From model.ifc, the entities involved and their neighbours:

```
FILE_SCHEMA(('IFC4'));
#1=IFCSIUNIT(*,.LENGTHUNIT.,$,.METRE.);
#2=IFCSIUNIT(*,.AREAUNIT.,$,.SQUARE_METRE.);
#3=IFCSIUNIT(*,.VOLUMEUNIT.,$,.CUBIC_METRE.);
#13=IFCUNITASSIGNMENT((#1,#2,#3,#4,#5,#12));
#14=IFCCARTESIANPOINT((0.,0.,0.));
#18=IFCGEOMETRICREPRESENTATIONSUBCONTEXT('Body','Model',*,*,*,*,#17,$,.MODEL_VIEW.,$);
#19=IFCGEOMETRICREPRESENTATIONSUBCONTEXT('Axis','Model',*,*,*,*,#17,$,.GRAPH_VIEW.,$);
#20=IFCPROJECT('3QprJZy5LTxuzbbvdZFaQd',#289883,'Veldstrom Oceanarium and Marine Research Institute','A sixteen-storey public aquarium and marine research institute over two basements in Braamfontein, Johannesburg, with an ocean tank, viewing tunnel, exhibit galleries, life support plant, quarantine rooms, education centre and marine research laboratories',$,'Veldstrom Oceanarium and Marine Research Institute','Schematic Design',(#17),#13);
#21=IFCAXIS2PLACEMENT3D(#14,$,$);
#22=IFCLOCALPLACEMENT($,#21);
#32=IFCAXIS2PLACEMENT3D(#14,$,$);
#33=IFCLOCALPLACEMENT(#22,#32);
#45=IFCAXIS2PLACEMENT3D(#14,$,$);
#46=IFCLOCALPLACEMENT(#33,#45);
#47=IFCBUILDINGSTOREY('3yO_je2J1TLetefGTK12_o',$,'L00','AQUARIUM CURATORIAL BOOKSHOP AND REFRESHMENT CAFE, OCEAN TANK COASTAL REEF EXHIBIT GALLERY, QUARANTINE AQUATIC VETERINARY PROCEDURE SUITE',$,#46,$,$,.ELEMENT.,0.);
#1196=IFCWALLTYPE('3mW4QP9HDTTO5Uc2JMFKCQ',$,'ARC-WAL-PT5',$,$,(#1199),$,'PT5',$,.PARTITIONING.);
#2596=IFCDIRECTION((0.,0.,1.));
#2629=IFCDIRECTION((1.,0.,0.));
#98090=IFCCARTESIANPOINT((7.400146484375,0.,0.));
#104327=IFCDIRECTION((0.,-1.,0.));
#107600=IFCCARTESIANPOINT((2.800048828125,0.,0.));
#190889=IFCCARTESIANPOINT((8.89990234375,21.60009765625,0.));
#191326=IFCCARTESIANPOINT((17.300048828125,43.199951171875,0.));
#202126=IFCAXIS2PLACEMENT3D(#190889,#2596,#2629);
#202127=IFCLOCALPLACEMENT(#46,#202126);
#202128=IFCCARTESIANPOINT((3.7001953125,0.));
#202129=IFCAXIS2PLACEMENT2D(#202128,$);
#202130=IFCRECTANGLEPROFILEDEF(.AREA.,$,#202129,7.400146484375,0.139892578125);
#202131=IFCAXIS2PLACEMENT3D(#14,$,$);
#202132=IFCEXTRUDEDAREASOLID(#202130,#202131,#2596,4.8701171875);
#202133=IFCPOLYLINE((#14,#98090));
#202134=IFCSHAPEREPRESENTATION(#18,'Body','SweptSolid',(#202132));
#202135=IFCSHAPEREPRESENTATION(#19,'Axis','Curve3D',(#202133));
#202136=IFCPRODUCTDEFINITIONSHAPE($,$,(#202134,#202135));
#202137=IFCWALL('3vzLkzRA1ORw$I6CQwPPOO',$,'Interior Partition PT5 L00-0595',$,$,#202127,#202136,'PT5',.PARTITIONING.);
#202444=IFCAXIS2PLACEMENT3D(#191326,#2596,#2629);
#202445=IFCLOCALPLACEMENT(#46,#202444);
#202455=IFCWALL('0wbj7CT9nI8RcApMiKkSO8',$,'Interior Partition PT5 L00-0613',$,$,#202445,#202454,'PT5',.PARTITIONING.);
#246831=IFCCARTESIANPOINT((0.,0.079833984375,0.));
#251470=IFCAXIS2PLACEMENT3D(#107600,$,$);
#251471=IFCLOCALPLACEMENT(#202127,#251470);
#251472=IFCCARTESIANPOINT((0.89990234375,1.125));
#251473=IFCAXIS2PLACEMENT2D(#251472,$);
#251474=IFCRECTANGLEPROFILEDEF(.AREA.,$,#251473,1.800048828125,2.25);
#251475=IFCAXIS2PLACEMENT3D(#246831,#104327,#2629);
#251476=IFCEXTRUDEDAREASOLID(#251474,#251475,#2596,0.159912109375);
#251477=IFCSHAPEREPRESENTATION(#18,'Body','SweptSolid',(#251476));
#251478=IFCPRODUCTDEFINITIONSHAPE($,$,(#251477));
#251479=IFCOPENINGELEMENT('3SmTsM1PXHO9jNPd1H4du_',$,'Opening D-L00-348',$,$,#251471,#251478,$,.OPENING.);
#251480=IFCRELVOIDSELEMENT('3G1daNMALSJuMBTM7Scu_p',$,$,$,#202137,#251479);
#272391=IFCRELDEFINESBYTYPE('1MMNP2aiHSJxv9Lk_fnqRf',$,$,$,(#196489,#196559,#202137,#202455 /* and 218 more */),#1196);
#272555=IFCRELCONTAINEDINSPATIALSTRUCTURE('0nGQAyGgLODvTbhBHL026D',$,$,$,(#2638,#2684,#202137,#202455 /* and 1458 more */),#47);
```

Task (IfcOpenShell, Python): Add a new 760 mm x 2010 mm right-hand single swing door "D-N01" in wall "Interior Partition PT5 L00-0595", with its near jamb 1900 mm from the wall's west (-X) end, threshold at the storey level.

```python
import numpy as np
import ifcopenshell
import ifcopenshell.api.feature
import ifcopenshell.api.geometry
import ifcopenshell.api.root
import ifcopenshell.api.spatial
import ifcopenshell.geom
import ifcopenshell.util.element
import ifcopenshell.util.placement
import ifcopenshell.util.representation
import ifcopenshell.util.shape
import ifcopenshell.util.unit

model = ifcopenshell.open("model.ifc")
unit_scale = ifcopenshell.util.unit.calculate_unit_scale(model)
settings = ifcopenshell.geom.settings()


def volume(element):
    """Net volume in cubic metres, openings subtracted."""
    shape = ifcopenshell.geom.create_shape(settings, element)
    return ifcopenshell.util.shape.get_volume(shape.geometry)


wall = model.by_id(202137)
storey = ifcopenshell.util.element.get_container(wall, ifc_class="IfcBuildingStorey")
context = ifcopenshell.util.representation.get_context(model, "Model", "Body", "MODEL_VIEW")
before = volume(wall)

width, height, from_end, sill = 0.76, 2.01, 1.9, 0.0  # metres

# The wall runs along its own X axis, and the end named is its -X end.
wall_shape = ifcopenshell.geom.create_shape(settings, wall)
x, y, z = ifcopenshell.util.shape.get_vertices(wall_shape.geometry).T
start = x.min() + from_end
face, thickness = float(y.min()), float(y.max() - y.min())
wall_matrix = ifcopenshell.util.placement.get_local_placement(wall.ObjectPlacement)
level = ifcopenshell.util.placement.get_local_placement(storey.ObjectPlacement)[2, 3]


def in_wall(x, y):
    """Placement at x, y metres in the wall's axes, at sill height."""
    matrix = wall_matrix.copy()
    matrix[:, 3] = wall_matrix @ np.array([x / unit_scale, y / unit_scale, 0.0, 1.0])
    matrix[2, 3] = level + sill / unit_scale
    return matrix


# Opening: a box that overshoots both wall faces by 50 mm.
opening = ifcopenshell.api.root.create_entity(model, ifc_class="IfcOpeningElement", predefined_type="OPENING")
box = ifcopenshell.api.geometry.add_wall_representation(
    model, context=context, length=width, height=height, thickness=thickness + 0.1
)
ifcopenshell.api.geometry.assign_representation(model, product=opening, representation=box)
ifcopenshell.api.geometry.edit_object_placement(model, product=opening, matrix=in_wall(start, face - 0.05), is_si=False)
ifcopenshell.api.feature.add_feature(model, feature=opening, element=wall)

door = ifcopenshell.api.root.create_entity(model, ifc_class="IfcDoor", name="D-N01", predefined_type="DOOR")
door.OverallWidth, door.OverallHeight = width / unit_scale, height / unit_scale
door.OperationType = "SINGLE_SWING_RIGHT"
body = ifcopenshell.api.geometry.add_door_representation(
    model,
    context=context,
    overall_width=door.OverallWidth,
    overall_height=door.OverallHeight,
    operation_type="SINGLE_SWING_RIGHT",
    lining_properties={"LiningDepth": thickness / unit_scale, "ThresholdDepth": thickness / unit_scale},
)
ifcopenshell.api.geometry.assign_representation(model, product=door, representation=body)
ifcopenshell.api.spatial.assign_container(model, products=[door], relating_structure=storey)
ifcopenshell.api.feature.add_filling(model, opening=opening, element=door)

# The lining spans the wall, so the door starts at the wall face.
ifcopenshell.api.geometry.edit_object_placement(model, product=door, matrix=in_wall(start, face), is_si=False)

after = volume(wall)

print(f"wall volume {before:.3f} -> {after:.3f} m3")

model.write("model-out.ifc")
```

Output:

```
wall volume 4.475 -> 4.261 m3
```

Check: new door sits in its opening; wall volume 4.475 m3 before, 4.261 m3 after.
